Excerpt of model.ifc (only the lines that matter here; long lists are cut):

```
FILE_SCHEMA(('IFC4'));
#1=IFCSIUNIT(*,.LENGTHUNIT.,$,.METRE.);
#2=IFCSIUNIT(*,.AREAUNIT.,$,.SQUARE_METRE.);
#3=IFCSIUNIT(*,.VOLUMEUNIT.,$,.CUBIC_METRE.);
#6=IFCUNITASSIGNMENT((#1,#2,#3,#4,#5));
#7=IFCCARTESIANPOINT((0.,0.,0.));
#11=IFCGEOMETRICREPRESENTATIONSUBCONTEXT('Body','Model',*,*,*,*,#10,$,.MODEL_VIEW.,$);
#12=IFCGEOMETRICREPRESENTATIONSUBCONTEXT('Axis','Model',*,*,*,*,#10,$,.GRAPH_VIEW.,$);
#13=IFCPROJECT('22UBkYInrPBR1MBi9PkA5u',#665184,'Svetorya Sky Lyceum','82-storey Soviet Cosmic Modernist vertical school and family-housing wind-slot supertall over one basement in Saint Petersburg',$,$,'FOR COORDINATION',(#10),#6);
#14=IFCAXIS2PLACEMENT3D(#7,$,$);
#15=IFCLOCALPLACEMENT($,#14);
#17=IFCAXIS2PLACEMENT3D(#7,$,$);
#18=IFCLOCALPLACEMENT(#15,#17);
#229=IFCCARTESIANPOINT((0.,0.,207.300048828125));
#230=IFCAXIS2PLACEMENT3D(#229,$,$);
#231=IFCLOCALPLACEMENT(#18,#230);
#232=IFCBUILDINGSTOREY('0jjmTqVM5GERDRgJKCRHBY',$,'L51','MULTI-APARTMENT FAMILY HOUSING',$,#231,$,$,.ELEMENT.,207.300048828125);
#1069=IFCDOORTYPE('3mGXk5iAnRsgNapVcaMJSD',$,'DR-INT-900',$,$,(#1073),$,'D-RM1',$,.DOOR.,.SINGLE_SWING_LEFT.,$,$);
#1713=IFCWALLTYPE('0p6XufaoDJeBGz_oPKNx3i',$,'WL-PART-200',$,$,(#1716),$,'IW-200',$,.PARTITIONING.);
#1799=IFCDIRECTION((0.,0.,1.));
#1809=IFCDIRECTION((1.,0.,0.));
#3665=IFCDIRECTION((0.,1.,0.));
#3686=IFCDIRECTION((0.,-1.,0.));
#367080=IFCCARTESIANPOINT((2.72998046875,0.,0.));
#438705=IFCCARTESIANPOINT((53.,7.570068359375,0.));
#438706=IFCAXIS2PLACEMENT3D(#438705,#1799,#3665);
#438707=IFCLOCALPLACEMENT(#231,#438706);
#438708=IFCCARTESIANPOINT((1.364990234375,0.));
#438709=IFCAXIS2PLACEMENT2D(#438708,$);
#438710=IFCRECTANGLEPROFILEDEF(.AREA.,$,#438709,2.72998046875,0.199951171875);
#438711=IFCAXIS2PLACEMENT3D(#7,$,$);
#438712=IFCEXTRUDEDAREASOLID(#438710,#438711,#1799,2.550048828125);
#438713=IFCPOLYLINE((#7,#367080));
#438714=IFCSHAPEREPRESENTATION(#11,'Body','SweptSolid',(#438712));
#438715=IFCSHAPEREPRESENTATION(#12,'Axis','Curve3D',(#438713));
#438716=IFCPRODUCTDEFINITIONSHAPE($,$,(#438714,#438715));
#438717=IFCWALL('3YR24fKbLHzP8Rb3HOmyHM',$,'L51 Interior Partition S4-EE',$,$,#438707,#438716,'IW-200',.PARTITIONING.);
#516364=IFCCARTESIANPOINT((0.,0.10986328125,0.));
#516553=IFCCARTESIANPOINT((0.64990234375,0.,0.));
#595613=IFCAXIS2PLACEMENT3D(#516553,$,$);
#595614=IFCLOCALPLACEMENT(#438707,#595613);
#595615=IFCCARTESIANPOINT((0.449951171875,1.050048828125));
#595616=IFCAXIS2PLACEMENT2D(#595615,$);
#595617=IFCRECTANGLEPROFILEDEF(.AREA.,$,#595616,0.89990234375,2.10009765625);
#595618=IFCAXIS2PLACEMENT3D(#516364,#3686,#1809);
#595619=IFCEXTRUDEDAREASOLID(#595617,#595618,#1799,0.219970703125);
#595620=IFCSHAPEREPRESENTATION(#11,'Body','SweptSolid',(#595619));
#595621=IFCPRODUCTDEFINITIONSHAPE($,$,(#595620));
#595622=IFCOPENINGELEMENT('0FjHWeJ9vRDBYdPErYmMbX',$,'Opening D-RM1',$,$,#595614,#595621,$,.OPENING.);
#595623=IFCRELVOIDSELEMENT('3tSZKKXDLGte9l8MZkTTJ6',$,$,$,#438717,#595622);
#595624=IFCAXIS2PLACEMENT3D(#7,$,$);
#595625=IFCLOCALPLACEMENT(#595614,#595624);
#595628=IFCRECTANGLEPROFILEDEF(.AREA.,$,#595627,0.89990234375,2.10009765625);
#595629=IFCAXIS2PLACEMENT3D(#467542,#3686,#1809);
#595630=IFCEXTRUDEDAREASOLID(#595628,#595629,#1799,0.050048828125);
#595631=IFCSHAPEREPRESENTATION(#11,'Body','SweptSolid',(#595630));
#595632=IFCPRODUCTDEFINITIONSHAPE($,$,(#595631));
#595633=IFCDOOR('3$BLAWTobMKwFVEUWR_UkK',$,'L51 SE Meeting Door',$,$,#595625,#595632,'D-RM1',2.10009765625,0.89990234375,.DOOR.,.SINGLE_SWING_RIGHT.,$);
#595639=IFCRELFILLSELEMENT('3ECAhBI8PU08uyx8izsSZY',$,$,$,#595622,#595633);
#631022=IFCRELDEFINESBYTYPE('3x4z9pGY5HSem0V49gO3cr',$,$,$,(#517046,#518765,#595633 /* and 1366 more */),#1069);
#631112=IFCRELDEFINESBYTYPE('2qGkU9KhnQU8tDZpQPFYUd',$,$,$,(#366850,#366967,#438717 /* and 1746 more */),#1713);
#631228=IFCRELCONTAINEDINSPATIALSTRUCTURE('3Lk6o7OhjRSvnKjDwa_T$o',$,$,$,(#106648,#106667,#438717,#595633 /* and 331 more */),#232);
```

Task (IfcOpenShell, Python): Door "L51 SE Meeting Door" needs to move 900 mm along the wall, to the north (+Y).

```python
import ifcopenshell
import ifcopenshell.api.geometry
import ifcopenshell.util.placement
import ifcopenshell.util.unit

model = ifcopenshell.open("model.ifc")
unit_scale = ifcopenshell.util.unit.calculate_unit_scale(model)

door = model.by_id(595633)
opening = door.FillsVoids[0].RelatingOpeningElement
wall = opening.VoidsElements[0].RelatingBuildingElement

wall_matrix = ifcopenshell.util.placement.get_local_placement(wall.ObjectPlacement)
shift = wall_matrix[:3, 0] * 0.9 / unit_scale
before = ifcopenshell.util.placement.get_local_placement(door.ObjectPlacement)[:3, 3].copy()

# The door is placed relative to its opening, so it follows when the opening moves.
matrix = ifcopenshell.util.placement.get_local_placement(opening.ObjectPlacement)
matrix[:3, 3] += shift
ifcopenshell.api.geometry.edit_object_placement(
    model, product=opening, matrix=matrix, is_si=False, should_transform_children=True
)

after = ifcopenshell.util.placement.get_local_placement(door.ObjectPlacement)[:3, 3]
print("door moved by", (after - before).round(3) + 0.0)

model.write("model_rev.ifc")
```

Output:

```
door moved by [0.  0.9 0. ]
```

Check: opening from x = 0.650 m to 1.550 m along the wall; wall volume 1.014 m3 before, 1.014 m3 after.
